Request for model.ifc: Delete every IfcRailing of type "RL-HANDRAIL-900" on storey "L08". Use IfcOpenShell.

First a look at what the model holds.

```python
import ifcopenshell
import ifcopenshell.util.element

model = ifcopenshell.open("model.ifc")
print(model.schema)
storey = next(s for s in model.by_type("IfcBuildingStorey") if s.Name == "L08")
railings = [e for e in ifcopenshell.util.element.get_decomposition(storey) if e.is_a("IfcRailing")]
seen = {}
for e in railings:
    element_type = ifcopenshell.util.element.get_type(e)
    name = element_type.Name if element_type not in (None, e) else None
    seen[name] = seen.get(name, 0) + 1
for name, count in sorted(seen.items(), key=str):
    print(count, "x", name)
```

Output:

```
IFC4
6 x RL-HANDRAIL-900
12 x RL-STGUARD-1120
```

```python
import ifcopenshell
import ifcopenshell.api.root
import ifcopenshell.util.element

model = ifcopenshell.open("model.ifc")

storey = next(s for s in model.by_type("IfcBuildingStorey") if s.Name == "L08")
railings = [e for e in ifcopenshell.util.element.get_decomposition(storey) if e.is_a("IfcRailing")]
targets = [e for e in railings if (t := ifcopenshell.util.element.get_type(e)) not in (None, e) and t.Name == "RL-HANDRAIL-900"]

for e in targets:
    ifcopenshell.api.root.remove_product(model, product=e)
print(len(targets), "removed")

model.write("model_updated.ifc")
```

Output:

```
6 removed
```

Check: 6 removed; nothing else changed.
